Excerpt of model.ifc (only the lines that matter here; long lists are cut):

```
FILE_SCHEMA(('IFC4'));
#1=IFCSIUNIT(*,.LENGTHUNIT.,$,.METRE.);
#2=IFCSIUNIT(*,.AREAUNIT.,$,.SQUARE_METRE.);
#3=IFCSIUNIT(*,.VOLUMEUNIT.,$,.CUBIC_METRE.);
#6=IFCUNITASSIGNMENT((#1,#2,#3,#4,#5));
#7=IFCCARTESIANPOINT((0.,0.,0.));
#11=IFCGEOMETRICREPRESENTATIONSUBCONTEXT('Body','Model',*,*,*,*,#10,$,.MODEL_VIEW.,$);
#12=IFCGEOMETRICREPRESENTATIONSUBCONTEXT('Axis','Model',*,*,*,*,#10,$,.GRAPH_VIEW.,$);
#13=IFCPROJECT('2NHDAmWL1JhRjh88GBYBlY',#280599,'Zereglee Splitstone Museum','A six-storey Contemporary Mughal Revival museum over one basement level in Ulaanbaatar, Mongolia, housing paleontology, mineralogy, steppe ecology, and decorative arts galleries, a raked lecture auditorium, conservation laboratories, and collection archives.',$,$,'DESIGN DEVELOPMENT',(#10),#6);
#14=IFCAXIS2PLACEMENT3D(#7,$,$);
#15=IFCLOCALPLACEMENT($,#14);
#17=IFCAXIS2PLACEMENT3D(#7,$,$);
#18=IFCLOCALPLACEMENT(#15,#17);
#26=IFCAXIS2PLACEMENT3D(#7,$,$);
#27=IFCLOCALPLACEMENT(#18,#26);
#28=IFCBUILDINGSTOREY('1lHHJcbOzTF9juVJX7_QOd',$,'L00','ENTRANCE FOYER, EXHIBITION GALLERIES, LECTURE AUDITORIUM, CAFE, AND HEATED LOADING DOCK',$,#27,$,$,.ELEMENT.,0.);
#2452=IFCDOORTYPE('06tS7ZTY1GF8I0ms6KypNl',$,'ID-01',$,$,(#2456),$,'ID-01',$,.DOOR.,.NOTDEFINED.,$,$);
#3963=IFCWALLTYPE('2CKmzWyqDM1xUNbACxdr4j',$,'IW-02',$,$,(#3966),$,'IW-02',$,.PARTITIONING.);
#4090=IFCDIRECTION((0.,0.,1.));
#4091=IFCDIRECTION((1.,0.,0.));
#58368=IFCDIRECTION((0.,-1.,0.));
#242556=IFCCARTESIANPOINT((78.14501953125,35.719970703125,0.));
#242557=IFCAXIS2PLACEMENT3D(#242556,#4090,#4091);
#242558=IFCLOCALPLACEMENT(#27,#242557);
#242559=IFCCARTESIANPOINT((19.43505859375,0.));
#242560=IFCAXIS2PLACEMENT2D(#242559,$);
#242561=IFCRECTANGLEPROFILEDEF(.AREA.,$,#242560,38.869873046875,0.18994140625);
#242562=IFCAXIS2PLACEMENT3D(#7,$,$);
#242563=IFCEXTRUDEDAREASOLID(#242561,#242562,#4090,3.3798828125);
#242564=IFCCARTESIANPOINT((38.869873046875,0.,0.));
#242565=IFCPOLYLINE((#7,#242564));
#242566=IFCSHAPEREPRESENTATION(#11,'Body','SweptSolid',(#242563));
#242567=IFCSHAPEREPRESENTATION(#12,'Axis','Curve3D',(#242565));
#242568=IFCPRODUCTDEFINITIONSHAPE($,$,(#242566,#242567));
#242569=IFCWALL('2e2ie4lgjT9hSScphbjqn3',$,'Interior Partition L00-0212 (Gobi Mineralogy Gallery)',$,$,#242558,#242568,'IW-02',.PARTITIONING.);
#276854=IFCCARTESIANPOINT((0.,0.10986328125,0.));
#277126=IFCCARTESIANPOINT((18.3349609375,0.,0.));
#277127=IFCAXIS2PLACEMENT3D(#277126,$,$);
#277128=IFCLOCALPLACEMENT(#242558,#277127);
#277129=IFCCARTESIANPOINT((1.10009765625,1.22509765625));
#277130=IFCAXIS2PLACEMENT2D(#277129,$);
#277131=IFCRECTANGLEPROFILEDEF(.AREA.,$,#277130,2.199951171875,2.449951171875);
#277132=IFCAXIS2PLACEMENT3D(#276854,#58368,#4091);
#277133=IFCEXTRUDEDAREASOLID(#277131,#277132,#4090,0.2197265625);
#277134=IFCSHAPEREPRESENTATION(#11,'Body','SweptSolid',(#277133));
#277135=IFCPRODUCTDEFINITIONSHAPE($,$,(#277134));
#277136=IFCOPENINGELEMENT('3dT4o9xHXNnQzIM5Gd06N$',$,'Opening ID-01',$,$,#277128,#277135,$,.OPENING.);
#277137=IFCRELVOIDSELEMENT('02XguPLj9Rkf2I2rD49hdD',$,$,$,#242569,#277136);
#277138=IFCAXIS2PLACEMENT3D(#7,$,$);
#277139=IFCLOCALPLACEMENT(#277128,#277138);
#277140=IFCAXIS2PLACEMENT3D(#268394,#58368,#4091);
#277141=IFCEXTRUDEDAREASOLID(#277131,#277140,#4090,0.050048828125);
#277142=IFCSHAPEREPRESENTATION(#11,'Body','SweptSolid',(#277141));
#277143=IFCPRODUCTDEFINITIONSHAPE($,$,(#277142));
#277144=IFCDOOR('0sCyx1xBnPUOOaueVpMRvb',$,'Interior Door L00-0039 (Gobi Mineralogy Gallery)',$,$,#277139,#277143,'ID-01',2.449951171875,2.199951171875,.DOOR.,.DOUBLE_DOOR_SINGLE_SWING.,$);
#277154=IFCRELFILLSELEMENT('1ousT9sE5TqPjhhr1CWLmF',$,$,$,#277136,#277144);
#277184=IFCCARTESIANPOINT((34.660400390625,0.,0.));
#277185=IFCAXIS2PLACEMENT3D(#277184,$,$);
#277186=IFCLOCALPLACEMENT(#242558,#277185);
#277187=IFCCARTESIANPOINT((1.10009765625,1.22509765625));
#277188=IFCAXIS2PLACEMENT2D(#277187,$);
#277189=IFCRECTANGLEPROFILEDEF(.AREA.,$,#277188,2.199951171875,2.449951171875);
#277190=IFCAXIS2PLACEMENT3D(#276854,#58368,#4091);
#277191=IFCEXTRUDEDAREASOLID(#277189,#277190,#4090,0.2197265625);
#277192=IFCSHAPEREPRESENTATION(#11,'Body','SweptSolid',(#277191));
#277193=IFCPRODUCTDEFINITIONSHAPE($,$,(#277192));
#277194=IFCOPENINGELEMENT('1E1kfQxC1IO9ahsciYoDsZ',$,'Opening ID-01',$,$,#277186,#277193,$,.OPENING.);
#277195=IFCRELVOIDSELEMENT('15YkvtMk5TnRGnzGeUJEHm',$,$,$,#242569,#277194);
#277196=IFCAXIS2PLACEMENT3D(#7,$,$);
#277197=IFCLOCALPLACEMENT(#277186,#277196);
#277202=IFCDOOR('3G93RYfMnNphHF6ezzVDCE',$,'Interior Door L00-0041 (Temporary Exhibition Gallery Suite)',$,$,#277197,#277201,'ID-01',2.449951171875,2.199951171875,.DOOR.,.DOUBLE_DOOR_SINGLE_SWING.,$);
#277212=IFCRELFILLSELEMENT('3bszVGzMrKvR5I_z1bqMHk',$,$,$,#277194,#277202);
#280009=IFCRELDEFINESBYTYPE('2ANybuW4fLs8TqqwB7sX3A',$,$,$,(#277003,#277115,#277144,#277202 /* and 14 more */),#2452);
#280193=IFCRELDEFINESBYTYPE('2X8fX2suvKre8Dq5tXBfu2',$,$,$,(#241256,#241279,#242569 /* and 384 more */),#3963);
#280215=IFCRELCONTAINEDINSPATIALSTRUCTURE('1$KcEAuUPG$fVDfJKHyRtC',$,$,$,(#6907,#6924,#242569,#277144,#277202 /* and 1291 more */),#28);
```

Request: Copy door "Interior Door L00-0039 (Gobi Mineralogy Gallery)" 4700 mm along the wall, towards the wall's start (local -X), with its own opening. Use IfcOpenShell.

```python
import ifcopenshell
import ifcopenshell.api.feature
import ifcopenshell.api.geometry
import ifcopenshell.api.root
import ifcopenshell.geom
import ifcopenshell.util.element
import ifcopenshell.util.placement
import ifcopenshell.util.shape
import ifcopenshell.util.unit

model = ifcopenshell.open("model.ifc")
unit_scale = ifcopenshell.util.unit.calculate_unit_scale(model)
settings = ifcopenshell.geom.settings()


def volume(element):
    """Net volume in cubic metres, openings subtracted."""
    shape = ifcopenshell.geom.create_shape(settings, element)
    return ifcopenshell.util.shape.get_volume(shape.geometry)


door = model.by_id(277144)
opening = door.FillsVoids[0].RelatingOpeningElement
wall = opening.VoidsElements[0].RelatingBuildingElement
before = volume(wall)
shift = ifcopenshell.util.placement.get_local_placement(wall.ObjectPlacement)[:3, 0] * -4.7 / unit_scale

# copy_class copies the void relationship, type, container and properties, but no geometry.
new_opening = ifcopenshell.api.root.copy_class(model, product=opening)
new_opening.Representation = ifcopenshell.util.element.copy_deep(
    model, opening.Representation, exclude=["IfcGeometricRepresentationContext", "IfcRepresentationMap"]
)
new_door = ifcopenshell.api.root.copy_class(model, product=door)
new_door.Representation = ifcopenshell.util.element.copy_deep(
    model, door.Representation, exclude=["IfcGeometricRepresentationContext", "IfcRepresentationMap"]
)
new_door.Tag = None
ifcopenshell.api.feature.add_filling(model, opening=new_opening, element=new_door)

for old, new in ((opening, new_opening), (door, new_door)):
    matrix = ifcopenshell.util.placement.get_local_placement(old.ObjectPlacement)
    matrix[:3, 3] += shift
    ifcopenshell.api.geometry.edit_object_placement(model, product=new, matrix=matrix, is_si=False)

after = volume(wall)

print(f"wall volume {before:.3f} -> {after:.3f} m3")

model.write("model_edited.ifc")
```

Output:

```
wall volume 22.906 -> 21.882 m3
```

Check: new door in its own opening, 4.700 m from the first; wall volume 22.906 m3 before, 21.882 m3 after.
